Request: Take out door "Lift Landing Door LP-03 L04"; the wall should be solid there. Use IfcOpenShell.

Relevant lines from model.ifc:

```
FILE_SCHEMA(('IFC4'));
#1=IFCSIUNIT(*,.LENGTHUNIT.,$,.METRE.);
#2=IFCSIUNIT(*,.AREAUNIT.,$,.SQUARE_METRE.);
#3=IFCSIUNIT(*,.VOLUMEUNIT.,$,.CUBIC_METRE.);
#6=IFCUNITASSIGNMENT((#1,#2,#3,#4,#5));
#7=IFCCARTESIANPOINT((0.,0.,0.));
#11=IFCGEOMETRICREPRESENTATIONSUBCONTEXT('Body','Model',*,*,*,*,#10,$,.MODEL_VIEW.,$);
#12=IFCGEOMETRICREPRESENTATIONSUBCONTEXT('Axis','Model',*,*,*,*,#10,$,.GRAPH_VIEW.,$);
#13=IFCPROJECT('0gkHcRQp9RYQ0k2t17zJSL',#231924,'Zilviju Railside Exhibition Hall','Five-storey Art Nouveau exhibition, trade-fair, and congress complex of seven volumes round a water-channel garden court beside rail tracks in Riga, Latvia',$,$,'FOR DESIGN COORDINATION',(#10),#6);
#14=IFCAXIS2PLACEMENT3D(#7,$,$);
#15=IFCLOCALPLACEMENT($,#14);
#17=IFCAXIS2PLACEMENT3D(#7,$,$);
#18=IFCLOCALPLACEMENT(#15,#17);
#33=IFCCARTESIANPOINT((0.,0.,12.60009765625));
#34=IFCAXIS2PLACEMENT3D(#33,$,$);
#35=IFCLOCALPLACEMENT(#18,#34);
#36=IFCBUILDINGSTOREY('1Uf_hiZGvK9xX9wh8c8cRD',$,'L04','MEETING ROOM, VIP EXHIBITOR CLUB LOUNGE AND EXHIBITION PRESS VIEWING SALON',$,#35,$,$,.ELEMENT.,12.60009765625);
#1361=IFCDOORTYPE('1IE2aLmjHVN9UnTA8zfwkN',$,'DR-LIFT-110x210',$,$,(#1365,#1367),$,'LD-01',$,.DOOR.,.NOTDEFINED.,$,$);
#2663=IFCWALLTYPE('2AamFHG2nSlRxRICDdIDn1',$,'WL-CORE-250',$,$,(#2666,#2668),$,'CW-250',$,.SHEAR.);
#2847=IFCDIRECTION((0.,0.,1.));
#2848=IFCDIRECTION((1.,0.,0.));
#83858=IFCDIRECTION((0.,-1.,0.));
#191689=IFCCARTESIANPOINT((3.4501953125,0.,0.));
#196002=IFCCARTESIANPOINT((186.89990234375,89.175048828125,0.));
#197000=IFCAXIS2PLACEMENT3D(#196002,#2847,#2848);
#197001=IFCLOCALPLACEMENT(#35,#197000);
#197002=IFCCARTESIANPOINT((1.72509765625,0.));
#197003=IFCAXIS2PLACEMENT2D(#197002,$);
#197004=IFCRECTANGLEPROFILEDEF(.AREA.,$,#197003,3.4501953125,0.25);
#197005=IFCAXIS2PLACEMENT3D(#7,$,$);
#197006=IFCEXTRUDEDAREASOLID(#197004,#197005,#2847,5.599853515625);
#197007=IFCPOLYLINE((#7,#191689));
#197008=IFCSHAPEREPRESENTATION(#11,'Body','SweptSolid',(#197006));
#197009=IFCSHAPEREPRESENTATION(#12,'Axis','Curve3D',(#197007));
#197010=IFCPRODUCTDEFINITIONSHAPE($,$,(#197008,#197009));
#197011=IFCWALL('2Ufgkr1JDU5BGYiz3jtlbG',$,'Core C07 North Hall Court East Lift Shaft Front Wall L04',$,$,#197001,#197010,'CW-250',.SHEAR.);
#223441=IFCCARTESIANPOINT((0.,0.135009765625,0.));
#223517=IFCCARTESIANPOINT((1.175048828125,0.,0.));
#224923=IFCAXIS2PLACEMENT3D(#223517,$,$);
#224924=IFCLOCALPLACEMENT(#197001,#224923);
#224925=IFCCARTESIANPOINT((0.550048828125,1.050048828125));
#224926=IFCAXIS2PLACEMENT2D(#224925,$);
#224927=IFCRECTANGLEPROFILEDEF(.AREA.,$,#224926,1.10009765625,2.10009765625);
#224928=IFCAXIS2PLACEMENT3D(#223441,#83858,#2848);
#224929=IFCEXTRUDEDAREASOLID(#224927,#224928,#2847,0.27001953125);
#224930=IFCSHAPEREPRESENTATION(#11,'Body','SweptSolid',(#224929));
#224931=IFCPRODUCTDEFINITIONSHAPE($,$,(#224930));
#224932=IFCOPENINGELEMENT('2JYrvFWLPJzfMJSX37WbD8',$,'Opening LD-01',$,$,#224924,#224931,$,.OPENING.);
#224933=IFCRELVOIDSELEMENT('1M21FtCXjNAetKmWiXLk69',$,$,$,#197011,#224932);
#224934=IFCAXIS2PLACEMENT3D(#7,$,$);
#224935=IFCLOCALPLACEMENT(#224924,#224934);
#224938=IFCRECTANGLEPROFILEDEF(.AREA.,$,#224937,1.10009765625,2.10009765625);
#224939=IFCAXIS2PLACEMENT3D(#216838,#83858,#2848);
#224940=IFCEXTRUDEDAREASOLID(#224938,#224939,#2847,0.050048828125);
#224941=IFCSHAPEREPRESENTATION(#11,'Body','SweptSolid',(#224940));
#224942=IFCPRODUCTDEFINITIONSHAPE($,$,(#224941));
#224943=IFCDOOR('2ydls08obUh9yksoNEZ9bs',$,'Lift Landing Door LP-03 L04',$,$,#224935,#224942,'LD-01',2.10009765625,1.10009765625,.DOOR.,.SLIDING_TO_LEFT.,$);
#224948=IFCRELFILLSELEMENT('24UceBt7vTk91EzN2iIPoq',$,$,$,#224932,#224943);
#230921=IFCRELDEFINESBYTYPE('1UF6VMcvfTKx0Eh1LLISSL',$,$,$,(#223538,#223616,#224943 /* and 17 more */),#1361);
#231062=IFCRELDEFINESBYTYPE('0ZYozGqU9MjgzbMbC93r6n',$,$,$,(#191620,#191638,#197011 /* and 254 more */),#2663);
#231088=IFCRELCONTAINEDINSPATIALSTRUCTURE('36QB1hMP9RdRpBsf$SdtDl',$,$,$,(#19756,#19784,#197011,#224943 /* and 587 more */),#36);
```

```python
import ifcopenshell
import ifcopenshell.api.feature
import ifcopenshell.api.root
import ifcopenshell.geom
import ifcopenshell.util.shape

model = ifcopenshell.open("model.ifc")
settings = ifcopenshell.geom.settings()


def volume(element):
    """Net volume in cubic metres, openings subtracted."""
    shape = ifcopenshell.geom.create_shape(settings, element)
    return ifcopenshell.util.shape.get_volume(shape.geometry)


door = model.by_guid("2ydls08obUh9yksoNEZ9bs")
opening = door.FillsVoids[0].RelatingOpeningElement
wall = opening.VoidsElements[0].RelatingBuildingElement
before = volume(wall)

ifcopenshell.api.root.remove_product(model, product=door)
ifcopenshell.api.feature.remove_feature(model, feature=opening)

after = volume(wall)

print(f"wall volume {before:.3f} -> {after:.3f} m3")

model.write("model_v2.ifc")
```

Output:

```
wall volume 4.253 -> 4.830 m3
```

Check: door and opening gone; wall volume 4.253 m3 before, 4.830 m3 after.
